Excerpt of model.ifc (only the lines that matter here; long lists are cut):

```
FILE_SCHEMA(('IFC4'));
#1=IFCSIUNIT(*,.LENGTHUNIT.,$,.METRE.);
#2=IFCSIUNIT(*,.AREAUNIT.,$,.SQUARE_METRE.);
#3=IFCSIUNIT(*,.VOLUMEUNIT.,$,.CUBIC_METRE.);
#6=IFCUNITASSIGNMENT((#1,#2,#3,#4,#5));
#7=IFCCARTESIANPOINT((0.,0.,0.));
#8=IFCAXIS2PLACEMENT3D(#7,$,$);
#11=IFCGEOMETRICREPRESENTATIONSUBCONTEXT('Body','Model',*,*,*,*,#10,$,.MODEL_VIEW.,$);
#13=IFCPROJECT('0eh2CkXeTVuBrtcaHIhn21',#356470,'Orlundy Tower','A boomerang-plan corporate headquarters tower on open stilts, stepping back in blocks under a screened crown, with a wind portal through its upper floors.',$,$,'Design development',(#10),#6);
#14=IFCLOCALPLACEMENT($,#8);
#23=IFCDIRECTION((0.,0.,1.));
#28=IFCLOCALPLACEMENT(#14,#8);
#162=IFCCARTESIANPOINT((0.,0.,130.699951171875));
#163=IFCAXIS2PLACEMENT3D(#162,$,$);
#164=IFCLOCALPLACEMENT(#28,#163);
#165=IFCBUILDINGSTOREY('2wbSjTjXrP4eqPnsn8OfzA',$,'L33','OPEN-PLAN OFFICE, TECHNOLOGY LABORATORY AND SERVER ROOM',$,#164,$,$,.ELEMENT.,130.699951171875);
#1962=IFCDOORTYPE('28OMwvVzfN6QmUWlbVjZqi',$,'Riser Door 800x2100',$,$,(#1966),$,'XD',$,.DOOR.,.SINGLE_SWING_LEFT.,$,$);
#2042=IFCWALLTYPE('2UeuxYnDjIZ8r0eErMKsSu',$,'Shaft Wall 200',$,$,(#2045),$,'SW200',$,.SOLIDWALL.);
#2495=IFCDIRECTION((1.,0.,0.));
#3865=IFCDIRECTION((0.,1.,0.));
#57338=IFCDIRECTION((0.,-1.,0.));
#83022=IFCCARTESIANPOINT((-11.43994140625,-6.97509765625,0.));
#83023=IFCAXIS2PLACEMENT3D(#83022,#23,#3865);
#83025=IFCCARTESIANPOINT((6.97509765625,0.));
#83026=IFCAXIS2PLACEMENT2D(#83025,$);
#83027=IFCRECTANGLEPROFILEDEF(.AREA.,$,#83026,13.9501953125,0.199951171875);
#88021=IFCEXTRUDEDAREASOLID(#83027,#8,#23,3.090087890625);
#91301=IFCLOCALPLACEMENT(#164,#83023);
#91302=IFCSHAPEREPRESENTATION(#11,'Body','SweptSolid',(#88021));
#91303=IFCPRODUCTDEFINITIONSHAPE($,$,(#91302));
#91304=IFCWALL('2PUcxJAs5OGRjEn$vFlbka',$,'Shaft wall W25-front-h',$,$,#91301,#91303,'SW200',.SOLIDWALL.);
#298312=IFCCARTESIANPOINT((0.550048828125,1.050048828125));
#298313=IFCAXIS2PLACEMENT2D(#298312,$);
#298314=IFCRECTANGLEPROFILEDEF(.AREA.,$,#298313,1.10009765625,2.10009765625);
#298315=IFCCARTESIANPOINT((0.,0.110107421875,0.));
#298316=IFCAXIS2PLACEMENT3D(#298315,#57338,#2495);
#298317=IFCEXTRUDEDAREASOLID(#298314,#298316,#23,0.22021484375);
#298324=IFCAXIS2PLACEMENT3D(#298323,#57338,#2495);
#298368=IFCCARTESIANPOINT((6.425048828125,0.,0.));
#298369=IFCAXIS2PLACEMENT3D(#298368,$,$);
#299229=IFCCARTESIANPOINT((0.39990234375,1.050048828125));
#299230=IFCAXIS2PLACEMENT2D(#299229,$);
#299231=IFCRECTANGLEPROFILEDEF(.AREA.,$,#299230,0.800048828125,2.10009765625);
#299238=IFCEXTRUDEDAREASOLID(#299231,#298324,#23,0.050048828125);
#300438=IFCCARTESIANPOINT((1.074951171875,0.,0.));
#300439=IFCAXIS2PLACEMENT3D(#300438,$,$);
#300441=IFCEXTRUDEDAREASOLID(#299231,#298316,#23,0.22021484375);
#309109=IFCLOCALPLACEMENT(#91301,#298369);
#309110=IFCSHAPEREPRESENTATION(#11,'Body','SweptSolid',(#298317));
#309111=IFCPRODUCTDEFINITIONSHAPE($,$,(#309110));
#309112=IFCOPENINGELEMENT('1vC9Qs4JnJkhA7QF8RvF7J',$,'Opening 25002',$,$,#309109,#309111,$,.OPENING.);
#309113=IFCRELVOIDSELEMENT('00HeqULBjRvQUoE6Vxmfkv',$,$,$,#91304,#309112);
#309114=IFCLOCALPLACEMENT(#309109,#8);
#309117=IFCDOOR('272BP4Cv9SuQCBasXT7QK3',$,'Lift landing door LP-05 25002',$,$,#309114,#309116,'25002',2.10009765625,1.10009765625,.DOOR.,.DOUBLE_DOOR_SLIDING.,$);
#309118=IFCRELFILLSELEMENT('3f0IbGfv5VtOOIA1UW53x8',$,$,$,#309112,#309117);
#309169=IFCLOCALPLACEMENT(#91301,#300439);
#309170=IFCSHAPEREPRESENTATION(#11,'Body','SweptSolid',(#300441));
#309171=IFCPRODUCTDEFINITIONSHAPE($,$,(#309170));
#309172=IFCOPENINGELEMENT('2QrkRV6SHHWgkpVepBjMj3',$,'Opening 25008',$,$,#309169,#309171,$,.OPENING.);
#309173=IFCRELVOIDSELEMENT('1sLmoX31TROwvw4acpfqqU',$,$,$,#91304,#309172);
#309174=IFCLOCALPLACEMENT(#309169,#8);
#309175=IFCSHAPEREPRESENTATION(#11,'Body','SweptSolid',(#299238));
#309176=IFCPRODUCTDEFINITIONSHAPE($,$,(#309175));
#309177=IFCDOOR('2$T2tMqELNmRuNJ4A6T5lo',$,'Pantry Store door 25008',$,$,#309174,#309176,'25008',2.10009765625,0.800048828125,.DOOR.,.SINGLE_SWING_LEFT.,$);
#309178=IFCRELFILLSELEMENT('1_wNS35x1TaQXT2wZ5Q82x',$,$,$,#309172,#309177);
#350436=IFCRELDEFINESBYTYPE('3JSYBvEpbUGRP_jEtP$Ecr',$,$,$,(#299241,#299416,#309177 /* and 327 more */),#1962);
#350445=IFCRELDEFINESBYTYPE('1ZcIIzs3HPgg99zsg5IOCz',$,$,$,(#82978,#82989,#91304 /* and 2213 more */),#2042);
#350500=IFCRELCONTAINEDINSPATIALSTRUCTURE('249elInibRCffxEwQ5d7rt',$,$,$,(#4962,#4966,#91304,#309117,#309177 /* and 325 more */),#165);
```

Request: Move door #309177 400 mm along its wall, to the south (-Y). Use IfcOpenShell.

```python
import ifcopenshell
import ifcopenshell.api.geometry
import ifcopenshell.util.placement

model = ifcopenshell.open("model.ifc")

door = model.by_id(309177)
opening = door.FillsVoids[0].RelatingOpeningElement
wall = opening.VoidsElements[0].RelatingBuildingElement

wall_matrix = ifcopenshell.util.placement.get_local_placement(wall.ObjectPlacement)
shift = wall_matrix[:3, 0] * -0.4
before = ifcopenshell.util.placement.get_local_placement(door.ObjectPlacement)[:3, 3].copy()

# The door is placed relative to its opening, so it follows when the opening moves.
matrix = ifcopenshell.util.placement.get_local_placement(opening.ObjectPlacement)
matrix[:3, 3] += shift
ifcopenshell.api.geometry.edit_object_placement(
    model, product=opening, matrix=matrix, is_si=False, should_transform_children=True
)

after = ifcopenshell.util.placement.get_local_placement(door.ObjectPlacement)[:3, 3]
print("door moved by", (after - before).round(3) + 0.0)

model.write("model_rev.ifc")
```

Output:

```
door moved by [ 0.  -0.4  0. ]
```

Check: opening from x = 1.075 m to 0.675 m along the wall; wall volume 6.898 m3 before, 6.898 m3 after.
